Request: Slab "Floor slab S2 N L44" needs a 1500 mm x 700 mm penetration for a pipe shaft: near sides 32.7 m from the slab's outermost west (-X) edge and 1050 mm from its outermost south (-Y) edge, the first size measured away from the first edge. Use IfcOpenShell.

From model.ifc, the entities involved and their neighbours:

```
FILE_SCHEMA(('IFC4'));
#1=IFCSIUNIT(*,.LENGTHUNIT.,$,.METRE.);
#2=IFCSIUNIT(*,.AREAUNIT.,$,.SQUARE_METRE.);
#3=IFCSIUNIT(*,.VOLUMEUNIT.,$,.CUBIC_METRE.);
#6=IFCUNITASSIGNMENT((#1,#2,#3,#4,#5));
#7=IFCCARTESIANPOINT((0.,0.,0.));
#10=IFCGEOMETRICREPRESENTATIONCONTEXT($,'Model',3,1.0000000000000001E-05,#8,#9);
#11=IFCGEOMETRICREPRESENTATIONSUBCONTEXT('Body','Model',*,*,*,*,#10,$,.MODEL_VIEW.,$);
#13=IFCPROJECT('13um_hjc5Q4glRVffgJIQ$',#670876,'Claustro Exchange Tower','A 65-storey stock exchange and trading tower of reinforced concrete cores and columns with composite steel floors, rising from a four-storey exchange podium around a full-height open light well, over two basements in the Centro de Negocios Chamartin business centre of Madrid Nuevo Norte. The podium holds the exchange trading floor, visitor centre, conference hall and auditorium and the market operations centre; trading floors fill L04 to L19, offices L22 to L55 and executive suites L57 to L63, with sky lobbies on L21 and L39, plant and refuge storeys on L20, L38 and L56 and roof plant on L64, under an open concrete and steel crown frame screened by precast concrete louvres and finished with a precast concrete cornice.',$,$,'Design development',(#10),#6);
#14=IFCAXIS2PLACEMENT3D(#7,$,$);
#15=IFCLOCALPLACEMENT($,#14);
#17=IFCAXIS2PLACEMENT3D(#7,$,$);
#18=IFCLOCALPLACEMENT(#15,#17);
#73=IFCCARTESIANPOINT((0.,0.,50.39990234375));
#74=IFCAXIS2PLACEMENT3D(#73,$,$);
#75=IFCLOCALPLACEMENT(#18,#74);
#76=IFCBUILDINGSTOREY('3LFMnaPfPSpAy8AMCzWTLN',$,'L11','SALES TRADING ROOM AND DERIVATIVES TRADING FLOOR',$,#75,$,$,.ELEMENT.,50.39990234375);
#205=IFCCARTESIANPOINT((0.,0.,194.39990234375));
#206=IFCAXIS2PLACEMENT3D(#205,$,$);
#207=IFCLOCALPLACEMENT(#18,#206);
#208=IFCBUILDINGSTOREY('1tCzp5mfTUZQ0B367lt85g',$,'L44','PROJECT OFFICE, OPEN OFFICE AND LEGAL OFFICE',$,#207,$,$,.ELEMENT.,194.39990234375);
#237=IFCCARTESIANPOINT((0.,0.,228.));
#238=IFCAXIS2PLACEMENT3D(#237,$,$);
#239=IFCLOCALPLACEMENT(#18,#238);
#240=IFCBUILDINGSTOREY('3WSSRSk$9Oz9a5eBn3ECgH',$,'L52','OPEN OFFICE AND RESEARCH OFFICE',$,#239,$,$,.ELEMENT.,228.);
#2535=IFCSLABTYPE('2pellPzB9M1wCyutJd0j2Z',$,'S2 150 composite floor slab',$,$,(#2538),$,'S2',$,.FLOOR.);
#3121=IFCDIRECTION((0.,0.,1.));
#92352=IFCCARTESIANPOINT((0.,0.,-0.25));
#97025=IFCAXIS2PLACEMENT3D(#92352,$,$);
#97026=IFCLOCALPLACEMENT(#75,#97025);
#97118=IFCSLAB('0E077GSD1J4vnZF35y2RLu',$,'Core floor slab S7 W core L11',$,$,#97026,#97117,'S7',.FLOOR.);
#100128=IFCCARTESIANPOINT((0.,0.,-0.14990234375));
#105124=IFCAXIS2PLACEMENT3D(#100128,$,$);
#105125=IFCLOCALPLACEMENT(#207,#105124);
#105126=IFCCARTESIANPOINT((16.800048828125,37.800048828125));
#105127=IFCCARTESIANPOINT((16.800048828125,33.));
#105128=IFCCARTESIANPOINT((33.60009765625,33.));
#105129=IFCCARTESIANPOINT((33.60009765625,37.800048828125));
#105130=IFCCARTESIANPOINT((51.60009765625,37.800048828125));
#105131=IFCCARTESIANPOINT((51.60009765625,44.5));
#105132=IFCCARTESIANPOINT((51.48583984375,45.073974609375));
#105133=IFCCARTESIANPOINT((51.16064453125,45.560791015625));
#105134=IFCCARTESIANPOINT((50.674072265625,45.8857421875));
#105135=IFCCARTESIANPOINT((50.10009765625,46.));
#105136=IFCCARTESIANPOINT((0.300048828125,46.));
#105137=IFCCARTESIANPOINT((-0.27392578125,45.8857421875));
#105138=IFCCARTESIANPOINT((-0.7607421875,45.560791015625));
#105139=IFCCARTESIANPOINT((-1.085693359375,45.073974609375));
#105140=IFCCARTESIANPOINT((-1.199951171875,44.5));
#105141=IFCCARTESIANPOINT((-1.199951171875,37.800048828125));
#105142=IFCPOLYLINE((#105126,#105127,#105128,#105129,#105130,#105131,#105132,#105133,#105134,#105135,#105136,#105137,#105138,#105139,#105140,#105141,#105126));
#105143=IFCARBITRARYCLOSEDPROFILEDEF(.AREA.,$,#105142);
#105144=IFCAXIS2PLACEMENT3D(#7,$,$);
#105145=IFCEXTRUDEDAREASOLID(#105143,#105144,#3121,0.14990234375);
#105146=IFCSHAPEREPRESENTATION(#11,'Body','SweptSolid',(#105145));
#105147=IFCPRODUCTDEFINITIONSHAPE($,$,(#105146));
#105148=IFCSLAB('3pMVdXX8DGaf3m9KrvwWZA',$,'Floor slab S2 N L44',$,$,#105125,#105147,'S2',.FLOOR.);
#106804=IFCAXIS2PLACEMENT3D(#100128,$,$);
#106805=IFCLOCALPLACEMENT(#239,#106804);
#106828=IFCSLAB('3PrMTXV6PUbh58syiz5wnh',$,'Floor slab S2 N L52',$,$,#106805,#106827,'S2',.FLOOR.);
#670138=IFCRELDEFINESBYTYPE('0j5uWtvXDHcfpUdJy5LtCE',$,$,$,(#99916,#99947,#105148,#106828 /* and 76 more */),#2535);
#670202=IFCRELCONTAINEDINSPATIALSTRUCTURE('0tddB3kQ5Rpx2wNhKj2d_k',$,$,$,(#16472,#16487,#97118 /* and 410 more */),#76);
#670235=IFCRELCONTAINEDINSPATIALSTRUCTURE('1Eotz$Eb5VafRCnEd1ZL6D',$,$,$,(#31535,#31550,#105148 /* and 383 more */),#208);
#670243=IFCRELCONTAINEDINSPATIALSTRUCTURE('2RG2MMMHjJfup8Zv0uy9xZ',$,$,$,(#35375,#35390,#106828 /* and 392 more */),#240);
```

```python
import numpy as np
import ifcopenshell
import ifcopenshell.api.feature
import ifcopenshell.api.geometry
import ifcopenshell.api.root
import ifcopenshell.geom
import ifcopenshell.util.placement
import ifcopenshell.util.representation
import ifcopenshell.util.shape
import ifcopenshell.util.unit

model = ifcopenshell.open("model.ifc")
unit_scale = ifcopenshell.util.unit.calculate_unit_scale(model)
settings = ifcopenshell.geom.settings()


def volume(element):
    """Net volume in cubic metres, openings subtracted."""
    shape = ifcopenshell.geom.create_shape(settings, element)
    return ifcopenshell.util.shape.get_volume(shape.geometry)


slab = model.by_guid("3pMVdXX8DGaf3m9KrvwWZA")
before = volume(slab)

# Extent in the slab's own axes, in metres. The edges named are its -X and -Y sides.
slab_shape = ifcopenshell.geom.create_shape(settings, slab)
vertices = ifcopenshell.util.shape.get_vertices(slab_shape.geometry)
x_min, y_min, bottom = vertices.min(axis=0)
top = vertices[:, 2].max()

opening = ifcopenshell.api.root.create_entity(model, ifc_class="IfcOpeningElement", name="Pipe shaft opening", predefined_type="OPENING")
context = ifcopenshell.util.representation.get_context(model, "Model", "Body", "MODEL_VIEW")
width, depth = 1.5, 0.7
outline = [(0.0, 0.0), (width, 0.0), (width, depth), (0.0, depth), (0.0, 0.0)]
# Overshoot both faces by 50 mm so the cut is clean.
shape = ifcopenshell.api.geometry.add_slab_representation(
    model, context=context, depth=top - bottom + 0.1, polyline=outline
)
ifcopenshell.api.geometry.assign_representation(model, product=opening, representation=shape)

matrix = ifcopenshell.util.placement.get_local_placement(slab.ObjectPlacement)
matrix[:, 3] = matrix @ np.append(np.array([x_min + 32.7, y_min + 1.05, bottom - 0.05]) / unit_scale, 1.0)
ifcopenshell.api.geometry.edit_object_placement(model, product=opening, matrix=matrix, is_si=False)
ifcopenshell.api.feature.add_feature(model, feature=opening, element=slab)

after = volume(slab)

print(f"slab volume {before:.3f} -> {after:.3f} m3")

model.write("model-out.ifc")
```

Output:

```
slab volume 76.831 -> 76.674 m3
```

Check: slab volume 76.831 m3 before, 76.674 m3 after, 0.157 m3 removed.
